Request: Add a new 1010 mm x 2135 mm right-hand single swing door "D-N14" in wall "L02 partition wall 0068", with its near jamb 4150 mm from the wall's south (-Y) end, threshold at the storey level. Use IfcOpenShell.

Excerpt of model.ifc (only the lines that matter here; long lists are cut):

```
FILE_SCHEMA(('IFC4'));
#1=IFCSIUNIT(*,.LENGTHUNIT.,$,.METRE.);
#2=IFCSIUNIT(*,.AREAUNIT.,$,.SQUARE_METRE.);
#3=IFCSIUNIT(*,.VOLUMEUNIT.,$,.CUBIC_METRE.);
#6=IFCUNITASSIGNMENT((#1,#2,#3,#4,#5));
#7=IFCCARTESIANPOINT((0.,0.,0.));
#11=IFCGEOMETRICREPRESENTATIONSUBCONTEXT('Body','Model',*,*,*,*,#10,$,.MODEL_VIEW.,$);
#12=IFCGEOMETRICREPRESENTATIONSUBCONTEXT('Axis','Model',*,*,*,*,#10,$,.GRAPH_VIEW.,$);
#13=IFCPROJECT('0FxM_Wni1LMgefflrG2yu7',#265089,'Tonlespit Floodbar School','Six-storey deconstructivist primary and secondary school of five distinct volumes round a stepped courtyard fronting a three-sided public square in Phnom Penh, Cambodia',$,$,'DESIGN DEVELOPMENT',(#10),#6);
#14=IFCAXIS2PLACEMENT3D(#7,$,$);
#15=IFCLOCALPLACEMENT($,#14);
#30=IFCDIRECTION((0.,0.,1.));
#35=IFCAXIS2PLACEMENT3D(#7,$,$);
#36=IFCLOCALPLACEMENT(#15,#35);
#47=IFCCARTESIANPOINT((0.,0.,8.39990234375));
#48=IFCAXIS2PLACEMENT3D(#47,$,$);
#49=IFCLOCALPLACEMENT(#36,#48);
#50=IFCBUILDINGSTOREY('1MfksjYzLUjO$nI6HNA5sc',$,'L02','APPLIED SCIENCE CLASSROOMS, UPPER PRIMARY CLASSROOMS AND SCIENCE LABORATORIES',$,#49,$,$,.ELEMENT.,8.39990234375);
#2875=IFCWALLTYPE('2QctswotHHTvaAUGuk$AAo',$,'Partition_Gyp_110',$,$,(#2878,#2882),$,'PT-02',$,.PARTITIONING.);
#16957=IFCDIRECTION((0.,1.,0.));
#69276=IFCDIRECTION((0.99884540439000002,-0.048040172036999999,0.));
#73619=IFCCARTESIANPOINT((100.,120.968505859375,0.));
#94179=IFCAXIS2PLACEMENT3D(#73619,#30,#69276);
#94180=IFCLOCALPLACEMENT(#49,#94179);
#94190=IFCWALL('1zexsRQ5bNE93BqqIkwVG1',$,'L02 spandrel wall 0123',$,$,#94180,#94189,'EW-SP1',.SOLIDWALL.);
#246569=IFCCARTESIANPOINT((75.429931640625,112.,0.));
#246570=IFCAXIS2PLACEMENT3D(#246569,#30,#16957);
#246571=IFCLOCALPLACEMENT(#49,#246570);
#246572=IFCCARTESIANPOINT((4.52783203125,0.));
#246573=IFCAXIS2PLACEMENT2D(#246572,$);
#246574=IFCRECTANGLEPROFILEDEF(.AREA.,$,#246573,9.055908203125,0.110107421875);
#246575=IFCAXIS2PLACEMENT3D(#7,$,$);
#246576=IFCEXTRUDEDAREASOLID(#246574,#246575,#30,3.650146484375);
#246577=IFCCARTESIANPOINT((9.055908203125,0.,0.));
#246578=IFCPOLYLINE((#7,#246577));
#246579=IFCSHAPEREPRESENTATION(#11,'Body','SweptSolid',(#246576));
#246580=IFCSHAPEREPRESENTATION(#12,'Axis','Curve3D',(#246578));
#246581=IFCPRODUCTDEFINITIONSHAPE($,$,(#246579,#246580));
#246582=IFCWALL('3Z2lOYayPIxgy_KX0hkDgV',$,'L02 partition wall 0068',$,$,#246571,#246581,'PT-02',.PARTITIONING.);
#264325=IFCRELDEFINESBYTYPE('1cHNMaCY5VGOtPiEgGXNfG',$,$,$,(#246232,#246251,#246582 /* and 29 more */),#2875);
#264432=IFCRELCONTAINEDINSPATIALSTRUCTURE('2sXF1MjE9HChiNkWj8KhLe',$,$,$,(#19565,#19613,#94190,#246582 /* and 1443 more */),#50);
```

```python
import numpy as np
import ifcopenshell
import ifcopenshell.api.feature
import ifcopenshell.api.geometry
import ifcopenshell.api.root
import ifcopenshell.api.spatial
import ifcopenshell.geom
import ifcopenshell.util.element
import ifcopenshell.util.placement
import ifcopenshell.util.representation
import ifcopenshell.util.shape
import ifcopenshell.util.unit

model = ifcopenshell.open("model.ifc")
unit_scale = ifcopenshell.util.unit.calculate_unit_scale(model)
settings = ifcopenshell.geom.settings()


def volume(element):
    """Net volume in cubic metres, openings subtracted."""
    shape = ifcopenshell.geom.create_shape(settings, element)
    return ifcopenshell.util.shape.get_volume(shape.geometry)


wall = model.by_id(246582)
storey = ifcopenshell.util.element.get_container(wall, ifc_class="IfcBuildingStorey")
context = ifcopenshell.util.representation.get_context(model, "Model", "Body", "MODEL_VIEW")
before = volume(wall)

width, height, from_end, sill = 1.01, 2.135, 4.15, 0.0  # metres

# The wall runs along its own X axis, and the end named is its -X end.
wall_shape = ifcopenshell.geom.create_shape(settings, wall)
x, y, z = ifcopenshell.util.shape.get_vertices(wall_shape.geometry).T
start = x.min() + from_end
face, thickness = float(y.min()), float(y.max() - y.min())
wall_matrix = ifcopenshell.util.placement.get_local_placement(wall.ObjectPlacement)
level = ifcopenshell.util.placement.get_local_placement(storey.ObjectPlacement)[2, 3]


def in_wall(x, y):
    """Placement at x, y metres in the wall's axes, at sill height."""
    matrix = wall_matrix.copy()
    matrix[:, 3] = wall_matrix @ np.array([x / unit_scale, y / unit_scale, 0.0, 1.0])
    matrix[2, 3] = level + sill / unit_scale
    return matrix


# Opening: a box that overshoots both wall faces by 50 mm.
opening = ifcopenshell.api.root.create_entity(model, ifc_class="IfcOpeningElement", predefined_type="OPENING")
box = ifcopenshell.api.geometry.add_wall_representation(
    model, context=context, length=width, height=height, thickness=thickness + 0.1
)
ifcopenshell.api.geometry.assign_representation(model, product=opening, representation=box)
ifcopenshell.api.geometry.edit_object_placement(model, product=opening, matrix=in_wall(start, face - 0.05), is_si=False)
ifcopenshell.api.feature.add_feature(model, feature=opening, element=wall)

door = ifcopenshell.api.root.create_entity(model, ifc_class="IfcDoor", name="D-N14", predefined_type="DOOR")
door.OverallWidth, door.OverallHeight = width / unit_scale, height / unit_scale
door.OperationType = "SINGLE_SWING_RIGHT"
body = ifcopenshell.api.geometry.add_door_representation(
    model,
    context=context,
    overall_width=door.OverallWidth,
    overall_height=door.OverallHeight,
    operation_type="SINGLE_SWING_RIGHT",
    lining_properties={"LiningDepth": thickness / unit_scale, "ThresholdDepth": thickness / unit_scale},
)
ifcopenshell.api.geometry.assign_representation(model, product=door, representation=body)
ifcopenshell.api.spatial.assign_container(model, products=[door], relating_structure=storey)
ifcopenshell.api.feature.add_filling(model, opening=opening, element=door)

# The lining spans the wall, so the door starts at the wall face.
ifcopenshell.api.geometry.edit_object_placement(model, product=door, matrix=in_wall(start, face), is_si=False)

after = volume(wall)

print(f"wall volume {before:.3f} -> {after:.3f} m3")

model.write("model-out.ifc")
```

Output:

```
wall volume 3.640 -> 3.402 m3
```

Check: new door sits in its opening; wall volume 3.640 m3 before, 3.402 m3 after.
